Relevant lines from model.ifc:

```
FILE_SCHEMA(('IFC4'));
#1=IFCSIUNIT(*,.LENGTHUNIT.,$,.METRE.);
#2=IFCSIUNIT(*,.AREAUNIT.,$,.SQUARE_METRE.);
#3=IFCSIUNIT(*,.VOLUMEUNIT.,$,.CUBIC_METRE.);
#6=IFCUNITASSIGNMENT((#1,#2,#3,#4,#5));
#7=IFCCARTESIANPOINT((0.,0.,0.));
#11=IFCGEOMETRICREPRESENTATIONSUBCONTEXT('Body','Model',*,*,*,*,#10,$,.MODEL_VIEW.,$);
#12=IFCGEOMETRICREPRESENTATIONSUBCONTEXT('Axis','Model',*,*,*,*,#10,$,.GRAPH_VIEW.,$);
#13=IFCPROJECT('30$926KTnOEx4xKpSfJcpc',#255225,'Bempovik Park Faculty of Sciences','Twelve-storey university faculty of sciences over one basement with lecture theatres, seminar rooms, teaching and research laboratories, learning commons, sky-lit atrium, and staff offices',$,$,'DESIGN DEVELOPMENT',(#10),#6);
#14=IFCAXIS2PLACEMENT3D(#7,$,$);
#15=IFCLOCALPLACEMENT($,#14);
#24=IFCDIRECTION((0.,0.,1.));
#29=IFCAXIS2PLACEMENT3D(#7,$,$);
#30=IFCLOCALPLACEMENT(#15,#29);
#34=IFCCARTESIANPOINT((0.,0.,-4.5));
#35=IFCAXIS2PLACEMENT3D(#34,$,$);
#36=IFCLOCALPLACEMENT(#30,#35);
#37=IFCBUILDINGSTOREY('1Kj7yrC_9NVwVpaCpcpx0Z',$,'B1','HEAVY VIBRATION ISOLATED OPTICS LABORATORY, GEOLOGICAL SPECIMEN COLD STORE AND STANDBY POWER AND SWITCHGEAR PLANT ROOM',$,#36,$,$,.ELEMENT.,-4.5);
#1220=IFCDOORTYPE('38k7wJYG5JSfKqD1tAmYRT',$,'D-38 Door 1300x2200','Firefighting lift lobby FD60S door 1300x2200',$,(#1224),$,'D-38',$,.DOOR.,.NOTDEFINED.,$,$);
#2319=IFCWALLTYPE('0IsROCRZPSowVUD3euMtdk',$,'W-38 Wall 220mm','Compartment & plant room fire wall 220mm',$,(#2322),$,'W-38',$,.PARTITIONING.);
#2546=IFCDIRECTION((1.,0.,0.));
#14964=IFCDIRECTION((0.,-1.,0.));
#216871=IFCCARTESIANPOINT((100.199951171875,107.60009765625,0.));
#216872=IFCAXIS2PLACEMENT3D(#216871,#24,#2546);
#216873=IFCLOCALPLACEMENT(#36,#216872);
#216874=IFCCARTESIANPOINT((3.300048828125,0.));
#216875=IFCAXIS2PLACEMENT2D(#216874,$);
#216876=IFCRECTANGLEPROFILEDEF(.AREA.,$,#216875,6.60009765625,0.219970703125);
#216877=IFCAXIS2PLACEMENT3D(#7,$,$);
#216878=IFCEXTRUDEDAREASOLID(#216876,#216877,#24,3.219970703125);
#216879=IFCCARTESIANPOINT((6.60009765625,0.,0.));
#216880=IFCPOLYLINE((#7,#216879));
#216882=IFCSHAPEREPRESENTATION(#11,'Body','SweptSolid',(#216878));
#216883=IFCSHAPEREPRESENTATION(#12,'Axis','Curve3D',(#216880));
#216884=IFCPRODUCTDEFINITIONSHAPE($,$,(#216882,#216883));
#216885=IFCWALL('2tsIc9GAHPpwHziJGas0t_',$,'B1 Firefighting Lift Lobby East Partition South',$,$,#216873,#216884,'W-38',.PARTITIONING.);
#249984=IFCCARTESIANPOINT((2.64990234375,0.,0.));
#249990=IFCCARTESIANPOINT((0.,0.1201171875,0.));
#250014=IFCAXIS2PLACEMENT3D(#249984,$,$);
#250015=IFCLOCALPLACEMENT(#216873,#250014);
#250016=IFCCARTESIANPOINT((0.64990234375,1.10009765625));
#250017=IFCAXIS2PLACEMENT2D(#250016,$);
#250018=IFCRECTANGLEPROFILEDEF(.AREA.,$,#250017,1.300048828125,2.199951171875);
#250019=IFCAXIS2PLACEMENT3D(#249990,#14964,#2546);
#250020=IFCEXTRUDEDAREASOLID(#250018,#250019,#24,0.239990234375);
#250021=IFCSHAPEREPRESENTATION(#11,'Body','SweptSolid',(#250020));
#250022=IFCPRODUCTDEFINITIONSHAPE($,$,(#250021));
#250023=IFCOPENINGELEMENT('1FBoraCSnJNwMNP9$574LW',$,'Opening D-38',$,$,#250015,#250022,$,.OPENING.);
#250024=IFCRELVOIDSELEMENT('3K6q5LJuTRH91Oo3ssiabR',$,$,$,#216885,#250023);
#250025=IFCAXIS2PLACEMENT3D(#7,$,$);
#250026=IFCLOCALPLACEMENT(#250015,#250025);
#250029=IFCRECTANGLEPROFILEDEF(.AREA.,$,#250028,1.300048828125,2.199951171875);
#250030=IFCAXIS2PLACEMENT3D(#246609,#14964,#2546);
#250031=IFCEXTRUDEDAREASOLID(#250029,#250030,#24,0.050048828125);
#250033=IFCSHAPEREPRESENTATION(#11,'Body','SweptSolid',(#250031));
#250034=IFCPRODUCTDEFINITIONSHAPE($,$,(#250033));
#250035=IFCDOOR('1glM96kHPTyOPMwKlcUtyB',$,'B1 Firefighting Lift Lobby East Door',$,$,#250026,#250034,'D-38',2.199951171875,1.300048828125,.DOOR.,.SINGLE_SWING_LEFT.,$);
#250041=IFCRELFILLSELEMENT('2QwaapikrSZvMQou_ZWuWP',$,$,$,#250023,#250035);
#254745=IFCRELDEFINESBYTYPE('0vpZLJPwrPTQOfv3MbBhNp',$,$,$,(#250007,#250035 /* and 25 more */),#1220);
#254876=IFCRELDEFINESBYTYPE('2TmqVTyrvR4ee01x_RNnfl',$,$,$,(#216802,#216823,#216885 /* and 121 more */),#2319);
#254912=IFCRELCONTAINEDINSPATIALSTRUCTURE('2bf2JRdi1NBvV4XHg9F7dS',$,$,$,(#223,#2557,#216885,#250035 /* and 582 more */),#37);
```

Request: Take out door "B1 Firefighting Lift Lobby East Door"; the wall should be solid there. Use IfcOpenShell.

```python
import ifcopenshell
import ifcopenshell.api.feature
import ifcopenshell.api.root
import ifcopenshell.geom
import ifcopenshell.util.shape

model = ifcopenshell.open("model.ifc")
settings = ifcopenshell.geom.settings()


def volume(element):
    """Net volume in cubic metres, openings subtracted."""
    shape = ifcopenshell.geom.create_shape(settings, element)
    return ifcopenshell.util.shape.get_volume(shape.geometry)


door = model.by_guid("1glM96kHPTyOPMwKlcUtyB")
opening = door.FillsVoids[0].RelatingOpeningElement
wall = opening.VoidsElements[0].RelatingBuildingElement
before = volume(wall)

ifcopenshell.api.root.remove_product(model, product=door)
ifcopenshell.api.feature.remove_feature(model, feature=opening)

after = volume(wall)

print(f"wall volume {before:.3f} -> {after:.3f} m3")

model.write("model_updated.ifc")
```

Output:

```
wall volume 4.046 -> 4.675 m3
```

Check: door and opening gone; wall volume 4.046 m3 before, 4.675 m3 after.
